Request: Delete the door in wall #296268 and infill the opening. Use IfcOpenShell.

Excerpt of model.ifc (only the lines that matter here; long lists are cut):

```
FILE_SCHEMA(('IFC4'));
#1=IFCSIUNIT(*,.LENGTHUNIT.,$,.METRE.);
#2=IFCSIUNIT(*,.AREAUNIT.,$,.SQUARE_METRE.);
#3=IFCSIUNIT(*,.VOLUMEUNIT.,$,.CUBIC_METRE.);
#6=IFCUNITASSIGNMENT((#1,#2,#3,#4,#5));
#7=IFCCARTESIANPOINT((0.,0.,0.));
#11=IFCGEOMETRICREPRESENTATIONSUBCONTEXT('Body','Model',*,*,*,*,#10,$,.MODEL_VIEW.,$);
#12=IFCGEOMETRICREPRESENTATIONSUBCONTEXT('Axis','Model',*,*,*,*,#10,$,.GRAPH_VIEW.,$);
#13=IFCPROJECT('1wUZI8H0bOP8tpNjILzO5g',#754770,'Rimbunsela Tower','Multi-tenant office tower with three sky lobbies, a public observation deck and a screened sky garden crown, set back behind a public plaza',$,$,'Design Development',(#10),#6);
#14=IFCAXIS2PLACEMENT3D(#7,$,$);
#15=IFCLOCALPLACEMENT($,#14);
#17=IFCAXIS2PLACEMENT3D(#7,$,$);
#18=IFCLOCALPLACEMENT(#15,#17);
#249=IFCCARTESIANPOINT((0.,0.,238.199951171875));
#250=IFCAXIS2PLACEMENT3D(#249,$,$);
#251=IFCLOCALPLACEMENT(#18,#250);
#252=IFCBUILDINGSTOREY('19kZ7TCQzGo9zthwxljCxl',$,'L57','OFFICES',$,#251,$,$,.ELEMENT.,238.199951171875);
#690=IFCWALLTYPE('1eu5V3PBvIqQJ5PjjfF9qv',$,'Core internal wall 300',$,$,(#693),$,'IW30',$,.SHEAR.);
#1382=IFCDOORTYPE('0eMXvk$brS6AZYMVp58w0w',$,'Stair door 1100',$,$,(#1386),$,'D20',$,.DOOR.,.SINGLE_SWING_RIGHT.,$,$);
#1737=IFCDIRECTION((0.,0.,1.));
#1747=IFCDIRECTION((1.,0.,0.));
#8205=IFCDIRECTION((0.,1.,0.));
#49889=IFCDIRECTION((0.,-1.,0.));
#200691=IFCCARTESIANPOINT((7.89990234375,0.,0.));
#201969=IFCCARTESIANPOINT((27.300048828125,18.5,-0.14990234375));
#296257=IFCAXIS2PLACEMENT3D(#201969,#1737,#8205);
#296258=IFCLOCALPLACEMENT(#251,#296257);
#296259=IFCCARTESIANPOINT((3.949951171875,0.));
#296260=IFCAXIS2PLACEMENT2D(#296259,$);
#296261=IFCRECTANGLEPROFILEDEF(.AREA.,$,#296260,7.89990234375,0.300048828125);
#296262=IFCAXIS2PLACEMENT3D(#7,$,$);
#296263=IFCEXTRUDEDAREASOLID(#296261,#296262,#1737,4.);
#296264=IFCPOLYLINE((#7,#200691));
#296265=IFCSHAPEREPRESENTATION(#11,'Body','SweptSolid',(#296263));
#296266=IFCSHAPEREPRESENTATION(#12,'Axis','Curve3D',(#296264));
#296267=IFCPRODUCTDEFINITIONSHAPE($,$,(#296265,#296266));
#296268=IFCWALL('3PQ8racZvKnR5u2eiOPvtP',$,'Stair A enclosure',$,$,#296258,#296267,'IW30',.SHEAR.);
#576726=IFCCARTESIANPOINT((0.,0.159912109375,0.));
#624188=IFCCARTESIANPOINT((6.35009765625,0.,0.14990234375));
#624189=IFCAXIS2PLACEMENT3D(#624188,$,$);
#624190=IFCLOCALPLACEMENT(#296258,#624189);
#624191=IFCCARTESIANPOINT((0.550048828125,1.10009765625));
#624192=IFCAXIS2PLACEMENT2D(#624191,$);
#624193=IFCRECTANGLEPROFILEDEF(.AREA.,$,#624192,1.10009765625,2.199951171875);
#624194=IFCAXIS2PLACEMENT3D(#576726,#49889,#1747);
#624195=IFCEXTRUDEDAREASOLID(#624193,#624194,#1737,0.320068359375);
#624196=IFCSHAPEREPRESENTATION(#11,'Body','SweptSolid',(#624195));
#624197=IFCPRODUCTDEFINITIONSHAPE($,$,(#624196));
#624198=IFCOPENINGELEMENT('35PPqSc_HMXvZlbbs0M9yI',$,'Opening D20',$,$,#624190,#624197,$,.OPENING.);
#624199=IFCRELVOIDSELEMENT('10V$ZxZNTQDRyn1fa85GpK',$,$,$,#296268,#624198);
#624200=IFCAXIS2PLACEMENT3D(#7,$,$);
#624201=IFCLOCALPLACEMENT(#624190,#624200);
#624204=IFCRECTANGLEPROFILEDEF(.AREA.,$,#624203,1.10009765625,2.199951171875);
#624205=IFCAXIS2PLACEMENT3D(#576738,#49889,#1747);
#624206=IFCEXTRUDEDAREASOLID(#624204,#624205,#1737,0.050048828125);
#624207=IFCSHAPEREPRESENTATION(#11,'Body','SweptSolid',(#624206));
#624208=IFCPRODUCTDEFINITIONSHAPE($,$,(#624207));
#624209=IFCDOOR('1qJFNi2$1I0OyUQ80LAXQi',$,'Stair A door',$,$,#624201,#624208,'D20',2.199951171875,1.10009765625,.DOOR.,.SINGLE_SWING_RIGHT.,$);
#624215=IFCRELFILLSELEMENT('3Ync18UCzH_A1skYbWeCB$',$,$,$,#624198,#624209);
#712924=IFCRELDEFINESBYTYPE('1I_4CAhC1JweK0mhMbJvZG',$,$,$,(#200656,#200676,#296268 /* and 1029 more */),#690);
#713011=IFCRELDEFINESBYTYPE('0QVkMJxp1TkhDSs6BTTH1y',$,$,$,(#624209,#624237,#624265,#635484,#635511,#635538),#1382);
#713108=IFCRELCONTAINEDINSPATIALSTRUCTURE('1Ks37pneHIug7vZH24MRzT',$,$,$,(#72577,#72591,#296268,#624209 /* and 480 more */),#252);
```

```python
import ifcopenshell
import ifcopenshell.api.feature
import ifcopenshell.api.root
import ifcopenshell.geom
import ifcopenshell.util.shape

model = ifcopenshell.open("model.ifc")
settings = ifcopenshell.geom.settings()


def volume(element):
    """Net volume in cubic metres, openings subtracted."""
    shape = ifcopenshell.geom.create_shape(settings, element)
    return ifcopenshell.util.shape.get_volume(shape.geometry)


door = model.by_guid("1qJFNi2$1I0OyUQ80LAXQi")
opening = door.FillsVoids[0].RelatingOpeningElement
wall = opening.VoidsElements[0].RelatingBuildingElement
before = volume(wall)

ifcopenshell.api.root.remove_product(model, product=door)
ifcopenshell.api.feature.remove_feature(model, feature=opening)

after = volume(wall)

print(f"wall volume {before:.3f} -> {after:.3f} m3")

model.write("model_rev.ifc")
```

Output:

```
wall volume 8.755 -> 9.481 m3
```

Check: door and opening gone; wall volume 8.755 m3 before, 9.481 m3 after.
